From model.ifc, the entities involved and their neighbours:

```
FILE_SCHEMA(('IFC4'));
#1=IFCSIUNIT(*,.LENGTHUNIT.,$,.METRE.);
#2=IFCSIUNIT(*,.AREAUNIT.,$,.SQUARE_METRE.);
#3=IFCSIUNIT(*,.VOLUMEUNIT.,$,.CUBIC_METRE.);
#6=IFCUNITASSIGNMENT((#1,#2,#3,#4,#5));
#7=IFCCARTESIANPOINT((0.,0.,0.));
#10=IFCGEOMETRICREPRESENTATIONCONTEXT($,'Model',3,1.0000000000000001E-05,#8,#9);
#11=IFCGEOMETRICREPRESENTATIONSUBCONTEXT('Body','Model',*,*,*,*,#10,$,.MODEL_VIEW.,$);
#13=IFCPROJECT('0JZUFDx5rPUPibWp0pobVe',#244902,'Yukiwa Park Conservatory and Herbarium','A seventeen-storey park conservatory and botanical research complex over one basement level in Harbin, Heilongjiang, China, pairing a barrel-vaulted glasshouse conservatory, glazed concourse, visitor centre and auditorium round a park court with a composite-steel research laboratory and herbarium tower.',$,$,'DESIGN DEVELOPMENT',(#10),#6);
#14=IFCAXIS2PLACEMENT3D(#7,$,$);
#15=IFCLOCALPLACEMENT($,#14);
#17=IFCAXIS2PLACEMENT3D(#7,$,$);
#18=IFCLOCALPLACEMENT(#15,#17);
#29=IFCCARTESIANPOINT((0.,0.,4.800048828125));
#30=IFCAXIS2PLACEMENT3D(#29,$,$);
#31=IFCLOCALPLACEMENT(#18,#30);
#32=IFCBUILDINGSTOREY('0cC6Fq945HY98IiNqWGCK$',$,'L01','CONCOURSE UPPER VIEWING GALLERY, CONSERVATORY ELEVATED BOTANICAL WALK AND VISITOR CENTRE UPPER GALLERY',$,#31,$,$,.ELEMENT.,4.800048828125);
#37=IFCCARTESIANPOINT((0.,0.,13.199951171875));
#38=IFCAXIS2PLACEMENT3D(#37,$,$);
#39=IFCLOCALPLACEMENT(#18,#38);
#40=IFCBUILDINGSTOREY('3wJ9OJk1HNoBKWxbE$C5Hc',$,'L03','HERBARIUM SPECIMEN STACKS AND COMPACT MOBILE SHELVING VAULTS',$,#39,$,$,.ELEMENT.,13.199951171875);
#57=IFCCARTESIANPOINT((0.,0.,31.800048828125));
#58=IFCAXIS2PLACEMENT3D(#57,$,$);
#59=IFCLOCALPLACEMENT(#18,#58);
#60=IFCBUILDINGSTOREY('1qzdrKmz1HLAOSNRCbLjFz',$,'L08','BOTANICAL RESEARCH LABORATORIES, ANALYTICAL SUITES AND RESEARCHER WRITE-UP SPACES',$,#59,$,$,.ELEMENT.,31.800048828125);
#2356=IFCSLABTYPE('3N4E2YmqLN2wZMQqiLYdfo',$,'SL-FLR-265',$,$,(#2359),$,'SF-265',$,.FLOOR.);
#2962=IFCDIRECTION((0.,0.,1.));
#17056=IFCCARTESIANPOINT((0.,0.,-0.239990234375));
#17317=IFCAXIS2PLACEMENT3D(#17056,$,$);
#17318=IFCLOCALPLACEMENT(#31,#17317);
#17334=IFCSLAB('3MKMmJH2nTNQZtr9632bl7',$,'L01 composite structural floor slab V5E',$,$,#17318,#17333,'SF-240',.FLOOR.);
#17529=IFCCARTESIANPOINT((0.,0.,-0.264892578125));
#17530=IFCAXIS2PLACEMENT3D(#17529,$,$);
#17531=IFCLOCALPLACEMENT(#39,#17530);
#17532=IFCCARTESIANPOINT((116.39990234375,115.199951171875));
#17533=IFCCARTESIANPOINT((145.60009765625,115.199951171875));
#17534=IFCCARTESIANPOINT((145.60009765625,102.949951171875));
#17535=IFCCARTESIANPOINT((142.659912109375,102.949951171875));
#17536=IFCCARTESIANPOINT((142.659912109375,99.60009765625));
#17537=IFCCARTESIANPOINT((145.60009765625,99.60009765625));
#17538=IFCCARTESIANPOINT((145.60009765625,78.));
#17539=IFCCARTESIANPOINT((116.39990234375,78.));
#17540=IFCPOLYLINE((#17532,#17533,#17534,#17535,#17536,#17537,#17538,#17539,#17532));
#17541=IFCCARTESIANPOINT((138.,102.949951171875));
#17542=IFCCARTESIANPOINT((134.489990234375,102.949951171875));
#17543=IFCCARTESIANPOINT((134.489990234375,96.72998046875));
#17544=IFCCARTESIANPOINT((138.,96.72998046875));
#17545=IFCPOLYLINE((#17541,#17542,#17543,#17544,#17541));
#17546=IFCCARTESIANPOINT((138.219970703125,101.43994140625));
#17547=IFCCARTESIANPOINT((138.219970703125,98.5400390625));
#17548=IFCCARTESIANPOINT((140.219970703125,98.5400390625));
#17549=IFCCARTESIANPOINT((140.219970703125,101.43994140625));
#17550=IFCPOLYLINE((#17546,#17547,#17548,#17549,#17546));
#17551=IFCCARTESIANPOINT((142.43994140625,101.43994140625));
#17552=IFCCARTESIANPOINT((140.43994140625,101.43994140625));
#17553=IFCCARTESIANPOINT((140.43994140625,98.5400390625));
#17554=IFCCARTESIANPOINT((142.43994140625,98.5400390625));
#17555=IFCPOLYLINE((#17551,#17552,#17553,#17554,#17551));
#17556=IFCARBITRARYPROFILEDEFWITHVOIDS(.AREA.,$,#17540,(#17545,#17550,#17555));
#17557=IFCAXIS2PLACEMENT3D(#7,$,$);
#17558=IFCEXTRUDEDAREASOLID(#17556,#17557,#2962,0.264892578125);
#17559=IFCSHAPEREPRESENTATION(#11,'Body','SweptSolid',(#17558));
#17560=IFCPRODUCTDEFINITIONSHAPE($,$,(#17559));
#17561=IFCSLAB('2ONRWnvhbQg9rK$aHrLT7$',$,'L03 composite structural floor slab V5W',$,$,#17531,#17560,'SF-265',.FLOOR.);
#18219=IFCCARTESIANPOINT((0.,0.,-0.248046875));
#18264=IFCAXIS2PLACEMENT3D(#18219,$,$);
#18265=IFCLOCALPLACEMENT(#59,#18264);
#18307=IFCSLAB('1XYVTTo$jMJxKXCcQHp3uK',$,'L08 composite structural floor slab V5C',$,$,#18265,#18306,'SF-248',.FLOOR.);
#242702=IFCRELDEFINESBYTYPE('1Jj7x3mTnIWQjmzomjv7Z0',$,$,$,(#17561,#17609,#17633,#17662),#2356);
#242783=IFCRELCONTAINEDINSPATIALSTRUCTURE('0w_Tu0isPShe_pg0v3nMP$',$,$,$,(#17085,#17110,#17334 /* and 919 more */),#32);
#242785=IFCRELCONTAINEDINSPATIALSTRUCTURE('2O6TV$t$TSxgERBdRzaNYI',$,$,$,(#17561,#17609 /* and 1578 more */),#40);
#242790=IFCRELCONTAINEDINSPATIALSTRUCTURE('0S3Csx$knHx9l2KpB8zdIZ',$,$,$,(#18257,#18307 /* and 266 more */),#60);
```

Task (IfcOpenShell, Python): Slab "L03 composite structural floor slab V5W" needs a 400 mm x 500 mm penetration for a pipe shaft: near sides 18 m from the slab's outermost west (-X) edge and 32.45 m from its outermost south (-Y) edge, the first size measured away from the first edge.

```python
import numpy as np
import ifcopenshell
import ifcopenshell.api.feature
import ifcopenshell.api.geometry
import ifcopenshell.api.root
import ifcopenshell.geom
import ifcopenshell.util.placement
import ifcopenshell.util.representation
import ifcopenshell.util.shape
import ifcopenshell.util.unit

model = ifcopenshell.open("model.ifc")
unit_scale = ifcopenshell.util.unit.calculate_unit_scale(model)
settings = ifcopenshell.geom.settings()


def volume(element):
    """Net volume in cubic metres, openings subtracted."""
    shape = ifcopenshell.geom.create_shape(settings, element)
    return ifcopenshell.util.shape.get_volume(shape.geometry)


slab = model.by_guid("2ONRWnvhbQg9rK$aHrLT7$")
before = volume(slab)

# Extent in the slab's own axes, in metres. The edges named are its -X and -Y sides.
slab_shape = ifcopenshell.geom.create_shape(settings, slab)
vertices = ifcopenshell.util.shape.get_vertices(slab_shape.geometry)
x_min, y_min, bottom = vertices.min(axis=0)
top = vertices[:, 2].max()

opening = ifcopenshell.api.root.create_entity(model, ifc_class="IfcOpeningElement", name="Pipe shaft opening", predefined_type="OPENING")
context = ifcopenshell.util.representation.get_context(model, "Model", "Body", "MODEL_VIEW")
width, depth = 0.4, 0.5
outline = [(0.0, 0.0), (width, 0.0), (width, depth), (0.0, depth), (0.0, 0.0)]
# Overshoot both faces by 50 mm so the cut is clean.
shape = ifcopenshell.api.geometry.add_slab_representation(
    model, context=context, depth=top - bottom + 0.1, polyline=outline
)
ifcopenshell.api.geometry.assign_representation(model, product=opening, representation=shape)

matrix = ifcopenshell.util.placement.get_local_placement(slab.ObjectPlacement)
matrix[:, 3] = matrix @ np.append(np.array([x_min + 18, y_min + 32.45, bottom - 0.05]) / unit_scale, 1.0)
ifcopenshell.api.geometry.edit_object_placement(model, product=opening, matrix=matrix, is_si=False)
ifcopenshell.api.feature.add_feature(model, feature=opening, element=slab)

after = volume(slab)

print(f"slab volume {before:.3f} -> {after:.3f} m3")

model.write("model_updated.ifc")
```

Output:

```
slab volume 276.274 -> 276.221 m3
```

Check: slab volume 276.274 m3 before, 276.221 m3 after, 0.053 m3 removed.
